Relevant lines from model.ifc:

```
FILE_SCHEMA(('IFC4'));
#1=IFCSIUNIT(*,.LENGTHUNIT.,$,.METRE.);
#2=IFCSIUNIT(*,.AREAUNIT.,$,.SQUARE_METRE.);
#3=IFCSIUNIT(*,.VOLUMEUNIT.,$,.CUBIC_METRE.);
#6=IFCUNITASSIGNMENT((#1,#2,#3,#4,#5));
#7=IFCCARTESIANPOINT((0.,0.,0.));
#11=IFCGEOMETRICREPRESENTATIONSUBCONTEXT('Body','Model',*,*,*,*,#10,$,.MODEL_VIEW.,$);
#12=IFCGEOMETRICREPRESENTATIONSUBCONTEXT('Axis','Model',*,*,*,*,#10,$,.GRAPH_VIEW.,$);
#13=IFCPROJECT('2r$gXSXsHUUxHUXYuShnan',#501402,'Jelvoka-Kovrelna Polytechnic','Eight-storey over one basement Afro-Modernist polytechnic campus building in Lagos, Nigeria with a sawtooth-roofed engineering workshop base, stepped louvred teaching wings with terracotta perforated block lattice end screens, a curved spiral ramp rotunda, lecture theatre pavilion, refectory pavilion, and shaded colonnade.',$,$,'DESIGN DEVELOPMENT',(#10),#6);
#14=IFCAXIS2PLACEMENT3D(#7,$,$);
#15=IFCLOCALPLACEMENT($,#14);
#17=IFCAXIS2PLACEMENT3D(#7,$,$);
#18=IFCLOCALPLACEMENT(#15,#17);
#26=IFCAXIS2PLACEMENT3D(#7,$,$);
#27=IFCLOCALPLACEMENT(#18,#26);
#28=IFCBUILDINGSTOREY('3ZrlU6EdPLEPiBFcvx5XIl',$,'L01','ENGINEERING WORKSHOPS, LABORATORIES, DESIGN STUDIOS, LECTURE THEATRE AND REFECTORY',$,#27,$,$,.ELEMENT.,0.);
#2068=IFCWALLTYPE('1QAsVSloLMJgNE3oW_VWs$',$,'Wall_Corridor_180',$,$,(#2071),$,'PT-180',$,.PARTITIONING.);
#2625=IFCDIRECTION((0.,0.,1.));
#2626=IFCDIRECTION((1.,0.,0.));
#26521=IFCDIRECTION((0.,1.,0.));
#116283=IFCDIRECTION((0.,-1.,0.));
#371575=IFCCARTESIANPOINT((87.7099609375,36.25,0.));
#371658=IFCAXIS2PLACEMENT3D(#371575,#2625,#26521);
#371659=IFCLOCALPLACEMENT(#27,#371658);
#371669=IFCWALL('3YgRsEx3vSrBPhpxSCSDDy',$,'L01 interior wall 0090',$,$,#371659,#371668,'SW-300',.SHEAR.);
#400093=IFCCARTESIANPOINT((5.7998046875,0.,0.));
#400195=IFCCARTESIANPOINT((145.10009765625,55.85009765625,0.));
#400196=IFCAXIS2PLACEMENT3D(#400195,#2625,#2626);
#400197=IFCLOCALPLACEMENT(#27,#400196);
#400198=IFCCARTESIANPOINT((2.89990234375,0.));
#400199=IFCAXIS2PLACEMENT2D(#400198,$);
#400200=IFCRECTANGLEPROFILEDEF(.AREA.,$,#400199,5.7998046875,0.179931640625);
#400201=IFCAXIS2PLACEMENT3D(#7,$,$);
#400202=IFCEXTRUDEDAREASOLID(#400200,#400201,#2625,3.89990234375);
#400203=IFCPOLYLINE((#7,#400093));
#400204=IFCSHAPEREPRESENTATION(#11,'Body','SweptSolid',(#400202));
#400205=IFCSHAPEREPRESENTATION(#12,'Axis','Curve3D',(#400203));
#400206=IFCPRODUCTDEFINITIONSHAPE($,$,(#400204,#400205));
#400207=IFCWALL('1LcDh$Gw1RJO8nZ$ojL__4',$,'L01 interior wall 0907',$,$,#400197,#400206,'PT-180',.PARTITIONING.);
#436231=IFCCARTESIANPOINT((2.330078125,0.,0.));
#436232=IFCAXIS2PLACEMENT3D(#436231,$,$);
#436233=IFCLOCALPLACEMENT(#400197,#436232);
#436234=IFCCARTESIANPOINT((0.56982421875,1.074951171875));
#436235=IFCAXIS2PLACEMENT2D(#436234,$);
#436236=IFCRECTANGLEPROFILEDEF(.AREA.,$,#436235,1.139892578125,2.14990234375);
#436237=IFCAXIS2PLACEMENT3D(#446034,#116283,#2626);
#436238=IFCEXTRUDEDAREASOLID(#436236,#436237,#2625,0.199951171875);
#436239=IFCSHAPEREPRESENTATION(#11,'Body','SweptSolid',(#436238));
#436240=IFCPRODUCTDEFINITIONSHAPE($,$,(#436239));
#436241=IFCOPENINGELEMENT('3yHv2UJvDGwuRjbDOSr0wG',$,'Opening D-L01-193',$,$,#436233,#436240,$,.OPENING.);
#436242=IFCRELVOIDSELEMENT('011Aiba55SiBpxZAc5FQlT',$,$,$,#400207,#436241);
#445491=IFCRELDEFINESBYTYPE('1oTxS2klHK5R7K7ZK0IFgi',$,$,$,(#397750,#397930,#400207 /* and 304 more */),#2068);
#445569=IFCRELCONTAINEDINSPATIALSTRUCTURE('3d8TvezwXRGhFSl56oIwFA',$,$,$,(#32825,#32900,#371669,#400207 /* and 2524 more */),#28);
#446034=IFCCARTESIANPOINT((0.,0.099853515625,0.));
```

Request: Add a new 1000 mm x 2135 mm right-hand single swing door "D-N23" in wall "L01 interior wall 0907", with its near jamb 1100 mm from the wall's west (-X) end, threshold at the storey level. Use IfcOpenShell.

```python
import numpy as np
import ifcopenshell
import ifcopenshell.api.feature
import ifcopenshell.api.geometry
import ifcopenshell.api.root
import ifcopenshell.api.spatial
import ifcopenshell.geom
import ifcopenshell.util.element
import ifcopenshell.util.placement
import ifcopenshell.util.representation
import ifcopenshell.util.shape
import ifcopenshell.util.unit

model = ifcopenshell.open("model.ifc")
unit_scale = ifcopenshell.util.unit.calculate_unit_scale(model)
settings = ifcopenshell.geom.settings()


def volume(element):
    """Net volume in cubic metres, openings subtracted."""
    shape = ifcopenshell.geom.create_shape(settings, element)
    return ifcopenshell.util.shape.get_volume(shape.geometry)


wall = model.by_id(400207)
storey = ifcopenshell.util.element.get_container(wall, ifc_class="IfcBuildingStorey")
context = ifcopenshell.util.representation.get_context(model, "Model", "Body", "MODEL_VIEW")
before = volume(wall)

width, height, from_end, sill = 1, 2.135, 1.1, 0.0  # metres

# The wall runs along its own X axis, and the end named is its -X end.
wall_shape = ifcopenshell.geom.create_shape(settings, wall)
x, y, z = ifcopenshell.util.shape.get_vertices(wall_shape.geometry).T
start = x.min() + from_end
face, thickness = float(y.min()), float(y.max() - y.min())
wall_matrix = ifcopenshell.util.placement.get_local_placement(wall.ObjectPlacement)
level = ifcopenshell.util.placement.get_local_placement(storey.ObjectPlacement)[2, 3]


def in_wall(x, y):
    """Placement at x, y metres in the wall's axes, at sill height."""
    matrix = wall_matrix.copy()
    matrix[:, 3] = wall_matrix @ np.array([x / unit_scale, y / unit_scale, 0.0, 1.0])
    matrix[2, 3] = level + sill / unit_scale
    return matrix


# Opening: a box that overshoots both wall faces by 50 mm.
opening = ifcopenshell.api.root.create_entity(model, ifc_class="IfcOpeningElement", predefined_type="OPENING")
box = ifcopenshell.api.geometry.add_wall_representation(
    model, context=context, length=width, height=height, thickness=thickness + 0.1
)
ifcopenshell.api.geometry.assign_representation(model, product=opening, representation=box)
ifcopenshell.api.geometry.edit_object_placement(model, product=opening, matrix=in_wall(start, face - 0.05), is_si=False)
ifcopenshell.api.feature.add_feature(model, feature=opening, element=wall)

door = ifcopenshell.api.root.create_entity(model, ifc_class="IfcDoor", name="D-N23", predefined_type="DOOR")
door.OverallWidth, door.OverallHeight = width / unit_scale, height / unit_scale
door.OperationType = "SINGLE_SWING_RIGHT"
body = ifcopenshell.api.geometry.add_door_representation(
    model,
    context=context,
    overall_width=door.OverallWidth,
    overall_height=door.OverallHeight,
    operation_type="SINGLE_SWING_RIGHT",
    lining_properties={"LiningDepth": thickness / unit_scale, "ThresholdDepth": thickness / unit_scale},
)
ifcopenshell.api.geometry.assign_representation(model, product=door, representation=body)
ifcopenshell.api.spatial.assign_container(model, products=[door], relating_structure=storey)
ifcopenshell.api.feature.add_filling(model, opening=opening, element=door)

# The lining spans the wall, so the door starts at the wall face.
ifcopenshell.api.geometry.edit_object_placement(model, product=door, matrix=in_wall(start, face), is_si=False)

after = volume(wall)

print(f"wall volume {before:.3f} -> {after:.3f} m3")

model.write("model_rev.ifc")
```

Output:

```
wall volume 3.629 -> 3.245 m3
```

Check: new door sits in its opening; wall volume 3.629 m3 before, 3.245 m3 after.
